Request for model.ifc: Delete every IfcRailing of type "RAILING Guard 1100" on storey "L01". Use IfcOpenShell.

First a look at what the model holds.

```python
import ifcopenshell
import ifcopenshell.util.element

model = ifcopenshell.open("model.ifc")
print(model.schema)
storey = next(s for s in model.by_type("IfcBuildingStorey") if s.Name == "L01")
railings = [e for e in ifcopenshell.util.element.get_decomposition(storey) if e.is_a("IfcRailing")]
seen = {}
for e in railings:
    element_type = ifcopenshell.util.element.get_type(e)
    name = element_type.Name if element_type not in (None, e) else None
    seen[name] = seen.get(name, 0) + 1
for name, count in sorted(seen.items(), key=str):
    print(count, "x", name)
```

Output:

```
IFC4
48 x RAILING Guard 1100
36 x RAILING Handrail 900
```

```python
import ifcopenshell
import ifcopenshell.api.root
import ifcopenshell.util.element

model = ifcopenshell.open("model.ifc")

storey = next(s for s in model.by_type("IfcBuildingStorey") if s.Name == "L01")
railings = [e for e in ifcopenshell.util.element.get_decomposition(storey) if e.is_a("IfcRailing")]
targets = [e for e in railings if (t := ifcopenshell.util.element.get_type(e)) not in (None, e) and t.Name == "RAILING Guard 1100"]

for e in targets:
    ifcopenshell.api.root.remove_product(model, product=e)
print(len(targets), "removed")

model.write("model_updated.ifc")
```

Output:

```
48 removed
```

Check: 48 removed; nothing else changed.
